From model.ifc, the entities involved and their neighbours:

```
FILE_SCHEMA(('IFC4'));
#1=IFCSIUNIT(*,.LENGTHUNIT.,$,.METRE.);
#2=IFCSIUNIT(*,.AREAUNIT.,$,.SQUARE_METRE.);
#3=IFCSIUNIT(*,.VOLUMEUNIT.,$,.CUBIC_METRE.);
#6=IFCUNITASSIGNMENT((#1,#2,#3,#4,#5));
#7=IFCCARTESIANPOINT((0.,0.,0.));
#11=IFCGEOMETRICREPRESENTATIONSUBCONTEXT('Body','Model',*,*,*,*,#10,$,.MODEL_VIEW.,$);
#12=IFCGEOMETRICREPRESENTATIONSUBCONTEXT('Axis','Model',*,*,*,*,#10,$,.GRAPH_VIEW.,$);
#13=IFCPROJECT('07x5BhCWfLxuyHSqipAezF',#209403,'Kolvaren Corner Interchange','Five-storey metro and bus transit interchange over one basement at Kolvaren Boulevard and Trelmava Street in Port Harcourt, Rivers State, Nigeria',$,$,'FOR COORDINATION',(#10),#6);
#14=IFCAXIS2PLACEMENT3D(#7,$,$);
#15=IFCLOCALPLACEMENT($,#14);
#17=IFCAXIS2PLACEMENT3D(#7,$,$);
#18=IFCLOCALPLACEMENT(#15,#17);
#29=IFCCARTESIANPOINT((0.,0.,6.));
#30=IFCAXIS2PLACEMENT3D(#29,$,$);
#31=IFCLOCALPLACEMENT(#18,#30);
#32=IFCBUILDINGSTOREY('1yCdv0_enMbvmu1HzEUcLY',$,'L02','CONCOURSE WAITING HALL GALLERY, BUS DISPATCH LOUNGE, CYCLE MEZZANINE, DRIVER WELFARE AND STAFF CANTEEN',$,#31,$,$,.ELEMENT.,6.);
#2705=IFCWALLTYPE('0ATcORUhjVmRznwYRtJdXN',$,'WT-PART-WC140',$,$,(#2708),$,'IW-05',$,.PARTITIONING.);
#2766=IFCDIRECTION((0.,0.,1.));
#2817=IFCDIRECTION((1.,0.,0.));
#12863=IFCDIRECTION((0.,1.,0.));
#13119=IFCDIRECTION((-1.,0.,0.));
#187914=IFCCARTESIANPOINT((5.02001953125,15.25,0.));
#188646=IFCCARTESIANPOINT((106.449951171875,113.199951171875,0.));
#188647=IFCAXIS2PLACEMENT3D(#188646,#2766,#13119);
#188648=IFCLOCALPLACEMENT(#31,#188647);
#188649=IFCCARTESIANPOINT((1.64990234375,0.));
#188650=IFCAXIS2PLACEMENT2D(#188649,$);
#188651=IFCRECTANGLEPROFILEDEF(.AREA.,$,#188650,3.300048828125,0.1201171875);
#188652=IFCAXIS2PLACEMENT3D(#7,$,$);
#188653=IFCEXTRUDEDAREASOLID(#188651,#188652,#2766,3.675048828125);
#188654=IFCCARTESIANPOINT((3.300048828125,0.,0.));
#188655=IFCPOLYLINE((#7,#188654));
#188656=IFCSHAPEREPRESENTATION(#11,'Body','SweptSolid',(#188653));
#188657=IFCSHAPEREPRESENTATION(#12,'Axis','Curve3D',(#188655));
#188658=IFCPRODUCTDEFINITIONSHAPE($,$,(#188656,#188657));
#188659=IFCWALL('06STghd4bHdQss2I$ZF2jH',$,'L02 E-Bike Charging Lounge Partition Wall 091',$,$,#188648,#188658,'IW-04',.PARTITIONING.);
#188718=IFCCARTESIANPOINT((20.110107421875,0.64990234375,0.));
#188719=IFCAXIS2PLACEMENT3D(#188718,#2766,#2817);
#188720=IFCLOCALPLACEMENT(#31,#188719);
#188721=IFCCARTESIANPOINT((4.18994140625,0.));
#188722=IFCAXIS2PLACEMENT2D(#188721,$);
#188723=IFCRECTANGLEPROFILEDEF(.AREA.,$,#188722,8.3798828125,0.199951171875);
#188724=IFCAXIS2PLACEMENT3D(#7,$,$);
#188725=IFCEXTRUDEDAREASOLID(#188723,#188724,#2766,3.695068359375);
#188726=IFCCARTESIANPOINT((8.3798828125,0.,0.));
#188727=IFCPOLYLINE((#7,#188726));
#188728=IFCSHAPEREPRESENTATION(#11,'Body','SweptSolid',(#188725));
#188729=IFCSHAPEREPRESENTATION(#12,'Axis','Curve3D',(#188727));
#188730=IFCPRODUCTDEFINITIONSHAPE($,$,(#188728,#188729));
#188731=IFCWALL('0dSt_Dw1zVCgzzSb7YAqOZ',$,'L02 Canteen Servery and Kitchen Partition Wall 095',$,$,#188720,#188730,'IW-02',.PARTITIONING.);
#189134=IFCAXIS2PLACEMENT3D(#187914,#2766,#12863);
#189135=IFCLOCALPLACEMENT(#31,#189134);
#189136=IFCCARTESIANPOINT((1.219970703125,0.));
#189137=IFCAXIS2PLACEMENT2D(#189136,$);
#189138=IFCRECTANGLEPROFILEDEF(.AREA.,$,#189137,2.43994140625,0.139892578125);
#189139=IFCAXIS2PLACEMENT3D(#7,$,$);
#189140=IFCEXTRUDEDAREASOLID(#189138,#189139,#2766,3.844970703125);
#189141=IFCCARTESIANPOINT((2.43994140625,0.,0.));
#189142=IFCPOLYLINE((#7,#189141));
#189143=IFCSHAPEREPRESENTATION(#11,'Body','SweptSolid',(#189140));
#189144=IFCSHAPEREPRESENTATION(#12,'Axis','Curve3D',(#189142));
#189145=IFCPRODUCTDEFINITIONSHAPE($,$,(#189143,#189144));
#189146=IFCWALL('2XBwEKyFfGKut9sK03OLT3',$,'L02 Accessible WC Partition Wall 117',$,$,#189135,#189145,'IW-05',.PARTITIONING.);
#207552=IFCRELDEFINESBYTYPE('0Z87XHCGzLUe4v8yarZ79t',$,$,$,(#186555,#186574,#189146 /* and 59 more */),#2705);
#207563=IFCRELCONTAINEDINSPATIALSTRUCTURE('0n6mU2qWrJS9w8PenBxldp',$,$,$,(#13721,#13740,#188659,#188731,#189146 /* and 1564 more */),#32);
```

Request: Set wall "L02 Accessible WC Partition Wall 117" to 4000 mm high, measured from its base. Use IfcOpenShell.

```python
import ifcopenshell
import ifcopenshell.geom
import ifcopenshell.util.representation
import ifcopenshell.util.shape
import ifcopenshell.util.unit

model = ifcopenshell.open("model.ifc")
unit_scale = ifcopenshell.util.unit.calculate_unit_scale(model)
settings = ifcopenshell.geom.settings()


def volume(element):
    """Net volume in cubic metres, openings subtracted."""
    shape = ifcopenshell.geom.create_shape(settings, element)
    return ifcopenshell.util.shape.get_volume(shape.geometry)


wall = model.by_id(189146)
before = volume(wall)

body = ifcopenshell.util.representation.get_representation(wall, "Model", "Body")
solid = body.Items[0]
old_height = solid.Depth
solid.Depth = 4 / unit_scale
after = volume(wall)

print(f"height {old_height:g} -> {solid.Depth:g}, volume {before:.3f} -> {after:.3f} m3")

model.write("model_rev.ifc")
```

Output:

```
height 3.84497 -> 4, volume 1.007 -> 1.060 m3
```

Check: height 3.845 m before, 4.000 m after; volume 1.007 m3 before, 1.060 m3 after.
